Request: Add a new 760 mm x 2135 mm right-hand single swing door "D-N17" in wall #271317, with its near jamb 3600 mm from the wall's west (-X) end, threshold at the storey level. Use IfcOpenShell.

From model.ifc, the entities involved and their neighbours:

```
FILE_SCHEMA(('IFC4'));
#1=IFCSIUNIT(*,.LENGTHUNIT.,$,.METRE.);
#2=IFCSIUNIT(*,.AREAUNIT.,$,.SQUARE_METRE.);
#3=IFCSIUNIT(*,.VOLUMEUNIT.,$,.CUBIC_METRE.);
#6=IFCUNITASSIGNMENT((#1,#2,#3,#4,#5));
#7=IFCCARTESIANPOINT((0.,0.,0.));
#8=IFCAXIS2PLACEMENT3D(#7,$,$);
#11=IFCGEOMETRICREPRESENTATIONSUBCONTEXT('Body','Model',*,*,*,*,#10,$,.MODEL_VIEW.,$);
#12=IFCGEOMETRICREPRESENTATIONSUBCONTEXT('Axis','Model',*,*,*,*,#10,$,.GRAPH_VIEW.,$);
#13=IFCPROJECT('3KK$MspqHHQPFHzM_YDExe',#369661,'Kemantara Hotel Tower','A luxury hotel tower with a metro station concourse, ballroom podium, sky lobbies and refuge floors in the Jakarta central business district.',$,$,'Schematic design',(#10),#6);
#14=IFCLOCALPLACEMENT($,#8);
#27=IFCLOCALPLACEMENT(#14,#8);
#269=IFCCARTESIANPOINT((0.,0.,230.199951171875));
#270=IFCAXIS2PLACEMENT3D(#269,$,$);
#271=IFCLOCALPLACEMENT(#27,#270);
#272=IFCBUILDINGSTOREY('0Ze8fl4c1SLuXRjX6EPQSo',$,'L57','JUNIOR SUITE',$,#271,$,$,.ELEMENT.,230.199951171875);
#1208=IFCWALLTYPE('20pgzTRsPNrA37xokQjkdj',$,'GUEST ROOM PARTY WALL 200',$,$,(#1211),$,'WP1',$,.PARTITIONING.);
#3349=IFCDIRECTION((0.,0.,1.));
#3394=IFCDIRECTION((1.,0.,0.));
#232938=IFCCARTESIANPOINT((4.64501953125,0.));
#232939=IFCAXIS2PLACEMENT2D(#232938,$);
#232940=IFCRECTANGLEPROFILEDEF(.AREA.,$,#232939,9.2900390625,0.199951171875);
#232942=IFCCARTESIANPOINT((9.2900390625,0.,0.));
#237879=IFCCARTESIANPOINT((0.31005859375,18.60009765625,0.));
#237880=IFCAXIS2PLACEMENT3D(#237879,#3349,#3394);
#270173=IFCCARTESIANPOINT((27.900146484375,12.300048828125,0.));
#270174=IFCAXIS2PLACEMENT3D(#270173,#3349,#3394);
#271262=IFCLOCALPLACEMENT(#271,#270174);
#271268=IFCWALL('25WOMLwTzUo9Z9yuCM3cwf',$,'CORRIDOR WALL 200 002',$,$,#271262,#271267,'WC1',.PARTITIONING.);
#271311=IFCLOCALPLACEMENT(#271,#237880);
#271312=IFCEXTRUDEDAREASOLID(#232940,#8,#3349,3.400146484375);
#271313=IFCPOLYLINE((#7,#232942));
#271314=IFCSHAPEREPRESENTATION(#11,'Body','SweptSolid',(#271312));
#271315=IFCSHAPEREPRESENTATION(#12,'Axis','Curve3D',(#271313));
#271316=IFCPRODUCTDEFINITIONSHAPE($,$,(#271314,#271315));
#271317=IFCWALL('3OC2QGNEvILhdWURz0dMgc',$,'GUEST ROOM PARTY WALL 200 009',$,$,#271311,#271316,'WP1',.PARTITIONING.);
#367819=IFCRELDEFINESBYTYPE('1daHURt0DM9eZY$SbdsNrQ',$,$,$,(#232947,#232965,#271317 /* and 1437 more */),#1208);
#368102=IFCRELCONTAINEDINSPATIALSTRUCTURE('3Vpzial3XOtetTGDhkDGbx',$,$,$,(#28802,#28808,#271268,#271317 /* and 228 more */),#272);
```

```python
import numpy as np
import ifcopenshell
import ifcopenshell.api.feature
import ifcopenshell.api.geometry
import ifcopenshell.api.root
import ifcopenshell.api.spatial
import ifcopenshell.geom
import ifcopenshell.util.element
import ifcopenshell.util.placement
import ifcopenshell.util.representation
import ifcopenshell.util.shape
import ifcopenshell.util.unit

model = ifcopenshell.open("model.ifc")
unit_scale = ifcopenshell.util.unit.calculate_unit_scale(model)
settings = ifcopenshell.geom.settings()


def volume(element):
    """Net volume in cubic metres, openings subtracted."""
    shape = ifcopenshell.geom.create_shape(settings, element)
    return ifcopenshell.util.shape.get_volume(shape.geometry)


wall = model.by_guid("3OC2QGNEvILhdWURz0dMgc")
storey = ifcopenshell.util.element.get_container(wall, ifc_class="IfcBuildingStorey")
context = ifcopenshell.util.representation.get_context(model, "Model", "Body", "MODEL_VIEW")
before = volume(wall)

width, height, from_end, sill = 0.76, 2.135, 3.6, 0.0  # metres

# The wall runs along its own X axis, and the end named is its -X end.
wall_shape = ifcopenshell.geom.create_shape(settings, wall)
x, y, z = ifcopenshell.util.shape.get_vertices(wall_shape.geometry).T
start = x.min() + from_end
face, thickness = float(y.min()), float(y.max() - y.min())
wall_matrix = ifcopenshell.util.placement.get_local_placement(wall.ObjectPlacement)
level = ifcopenshell.util.placement.get_local_placement(storey.ObjectPlacement)[2, 3]


def in_wall(x, y):
    """Placement at x, y metres in the wall's axes, at sill height."""
    matrix = wall_matrix.copy()
    matrix[:, 3] = wall_matrix @ np.array([x / unit_scale, y / unit_scale, 0.0, 1.0])
    matrix[2, 3] = level + sill / unit_scale
    return matrix


# Opening: a box that overshoots both wall faces by 50 mm.
opening = ifcopenshell.api.root.create_entity(model, ifc_class="IfcOpeningElement", predefined_type="OPENING")
box = ifcopenshell.api.geometry.add_wall_representation(
    model, context=context, length=width, height=height, thickness=thickness + 0.1
)
ifcopenshell.api.geometry.assign_representation(model, product=opening, representation=box)
ifcopenshell.api.geometry.edit_object_placement(model, product=opening, matrix=in_wall(start, face - 0.05), is_si=False)
ifcopenshell.api.feature.add_feature(model, feature=opening, element=wall)

door = ifcopenshell.api.root.create_entity(model, ifc_class="IfcDoor", name="D-N17", predefined_type="DOOR")
door.OverallWidth, door.OverallHeight = width / unit_scale, height / unit_scale
door.OperationType = "SINGLE_SWING_RIGHT"
body = ifcopenshell.api.geometry.add_door_representation(
    model,
    context=context,
    overall_width=door.OverallWidth,
    overall_height=door.OverallHeight,
    operation_type="SINGLE_SWING_RIGHT",
    lining_properties={"LiningDepth": thickness / unit_scale, "ThresholdDepth": thickness / unit_scale},
)
ifcopenshell.api.geometry.assign_representation(model, product=door, representation=body)
ifcopenshell.api.spatial.assign_container(model, products=[door], relating_structure=storey)
ifcopenshell.api.feature.add_filling(model, opening=opening, element=door)

# The lining spans the wall, so the door starts at the wall face.
ifcopenshell.api.geometry.edit_object_placement(model, product=door, matrix=in_wall(start, face), is_si=False)

after = volume(wall)

print(f"wall volume {before:.3f} -> {after:.3f} m3")

model.write("model_updated.ifc")
```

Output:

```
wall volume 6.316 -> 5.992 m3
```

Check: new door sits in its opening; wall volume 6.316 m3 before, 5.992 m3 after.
